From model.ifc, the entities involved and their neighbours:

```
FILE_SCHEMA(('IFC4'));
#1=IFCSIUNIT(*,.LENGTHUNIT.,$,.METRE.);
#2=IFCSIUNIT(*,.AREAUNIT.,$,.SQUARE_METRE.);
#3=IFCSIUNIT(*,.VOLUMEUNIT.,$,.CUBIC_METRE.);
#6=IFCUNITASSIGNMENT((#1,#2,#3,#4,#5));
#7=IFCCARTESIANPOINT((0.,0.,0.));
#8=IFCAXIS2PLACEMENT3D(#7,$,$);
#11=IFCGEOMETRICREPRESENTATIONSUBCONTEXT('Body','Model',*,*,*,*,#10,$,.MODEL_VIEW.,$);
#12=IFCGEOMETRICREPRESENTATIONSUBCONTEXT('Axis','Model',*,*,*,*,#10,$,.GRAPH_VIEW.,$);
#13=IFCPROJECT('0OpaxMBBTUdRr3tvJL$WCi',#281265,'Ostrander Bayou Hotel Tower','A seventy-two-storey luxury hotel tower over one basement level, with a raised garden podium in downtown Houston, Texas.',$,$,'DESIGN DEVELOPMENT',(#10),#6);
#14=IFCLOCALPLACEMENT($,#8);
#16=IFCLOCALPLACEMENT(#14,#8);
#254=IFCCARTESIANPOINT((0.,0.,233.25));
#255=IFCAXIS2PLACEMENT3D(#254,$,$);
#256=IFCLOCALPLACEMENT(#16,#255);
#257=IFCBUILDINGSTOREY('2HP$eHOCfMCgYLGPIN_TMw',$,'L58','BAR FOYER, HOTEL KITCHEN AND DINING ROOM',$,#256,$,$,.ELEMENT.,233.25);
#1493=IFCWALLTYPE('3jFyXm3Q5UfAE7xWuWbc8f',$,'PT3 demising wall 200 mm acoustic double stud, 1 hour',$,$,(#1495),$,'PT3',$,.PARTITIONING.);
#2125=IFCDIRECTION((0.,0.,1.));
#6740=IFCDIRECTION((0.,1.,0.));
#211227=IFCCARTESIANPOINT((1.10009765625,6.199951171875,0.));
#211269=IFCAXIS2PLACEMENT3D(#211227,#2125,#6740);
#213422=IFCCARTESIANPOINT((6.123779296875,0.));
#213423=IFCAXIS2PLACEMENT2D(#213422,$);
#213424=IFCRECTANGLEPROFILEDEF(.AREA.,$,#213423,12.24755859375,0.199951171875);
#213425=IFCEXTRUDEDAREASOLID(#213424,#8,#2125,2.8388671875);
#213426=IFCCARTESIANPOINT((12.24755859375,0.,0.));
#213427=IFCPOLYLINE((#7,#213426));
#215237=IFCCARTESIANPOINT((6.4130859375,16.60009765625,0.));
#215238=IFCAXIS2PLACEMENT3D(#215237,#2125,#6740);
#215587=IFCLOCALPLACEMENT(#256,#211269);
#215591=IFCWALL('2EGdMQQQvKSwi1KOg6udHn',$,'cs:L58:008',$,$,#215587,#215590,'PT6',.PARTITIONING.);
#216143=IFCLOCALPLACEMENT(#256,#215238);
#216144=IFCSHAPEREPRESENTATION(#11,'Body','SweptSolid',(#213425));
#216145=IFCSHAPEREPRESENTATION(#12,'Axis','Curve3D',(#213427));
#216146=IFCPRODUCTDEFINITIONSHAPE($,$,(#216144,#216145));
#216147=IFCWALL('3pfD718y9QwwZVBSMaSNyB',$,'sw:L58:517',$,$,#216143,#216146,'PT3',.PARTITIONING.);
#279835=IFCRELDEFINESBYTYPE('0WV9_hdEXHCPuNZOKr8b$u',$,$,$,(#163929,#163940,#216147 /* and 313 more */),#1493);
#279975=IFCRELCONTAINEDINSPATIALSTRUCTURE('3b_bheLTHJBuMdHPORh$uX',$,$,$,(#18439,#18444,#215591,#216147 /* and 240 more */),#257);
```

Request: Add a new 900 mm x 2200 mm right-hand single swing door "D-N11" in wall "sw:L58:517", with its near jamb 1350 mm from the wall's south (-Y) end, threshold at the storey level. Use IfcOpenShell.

```python
import numpy as np
import ifcopenshell
import ifcopenshell.api.feature
import ifcopenshell.api.geometry
import ifcopenshell.api.root
import ifcopenshell.api.spatial
import ifcopenshell.geom
import ifcopenshell.util.element
import ifcopenshell.util.placement
import ifcopenshell.util.representation
import ifcopenshell.util.shape
import ifcopenshell.util.unit

model = ifcopenshell.open("model.ifc")
unit_scale = ifcopenshell.util.unit.calculate_unit_scale(model)
settings = ifcopenshell.geom.settings()


def volume(element):
    """Net volume in cubic metres, openings subtracted."""
    shape = ifcopenshell.geom.create_shape(settings, element)
    return ifcopenshell.util.shape.get_volume(shape.geometry)


wall = model.by_guid("3pfD718y9QwwZVBSMaSNyB")
storey = ifcopenshell.util.element.get_container(wall, ifc_class="IfcBuildingStorey")
context = ifcopenshell.util.representation.get_context(model, "Model", "Body", "MODEL_VIEW")
before = volume(wall)

width, height, from_end, sill = 0.9, 2.2, 1.35, 0.0  # metres

# The wall runs along its own X axis, and the end named is its -X end.
wall_shape = ifcopenshell.geom.create_shape(settings, wall)
x, y, z = ifcopenshell.util.shape.get_vertices(wall_shape.geometry).T
start = x.min() + from_end
face, thickness = float(y.min()), float(y.max() - y.min())
wall_matrix = ifcopenshell.util.placement.get_local_placement(wall.ObjectPlacement)
level = ifcopenshell.util.placement.get_local_placement(storey.ObjectPlacement)[2, 3]


def in_wall(x, y):
    """Placement at x, y metres in the wall's axes, at sill height."""
    matrix = wall_matrix.copy()
    matrix[:, 3] = wall_matrix @ np.array([x / unit_scale, y / unit_scale, 0.0, 1.0])
    matrix[2, 3] = level + sill / unit_scale
    return matrix


# Opening: a box that overshoots both wall faces by 50 mm.
opening = ifcopenshell.api.root.create_entity(model, ifc_class="IfcOpeningElement", predefined_type="OPENING")
box = ifcopenshell.api.geometry.add_wall_representation(
    model, context=context, length=width, height=height, thickness=thickness + 0.1
)
ifcopenshell.api.geometry.assign_representation(model, product=opening, representation=box)
ifcopenshell.api.geometry.edit_object_placement(model, product=opening, matrix=in_wall(start, face - 0.05), is_si=False)
ifcopenshell.api.feature.add_feature(model, feature=opening, element=wall)

door = ifcopenshell.api.root.create_entity(model, ifc_class="IfcDoor", name="D-N11", predefined_type="DOOR")
door.OverallWidth, door.OverallHeight = width / unit_scale, height / unit_scale
door.OperationType = "SINGLE_SWING_RIGHT"
body = ifcopenshell.api.geometry.add_door_representation(
    model,
    context=context,
    overall_width=door.OverallWidth,
    overall_height=door.OverallHeight,
    operation_type="SINGLE_SWING_RIGHT",
    lining_properties={"LiningDepth": thickness / unit_scale, "ThresholdDepth": thickness / unit_scale},
)
ifcopenshell.api.geometry.assign_representation(model, product=door, representation=body)
ifcopenshell.api.spatial.assign_container(model, products=[door], relating_structure=storey)
ifcopenshell.api.feature.add_filling(model, opening=opening, element=door)

# The lining spans the wall, so the door starts at the wall face.
ifcopenshell.api.geometry.edit_object_placement(model, product=door, matrix=in_wall(start, face), is_si=False)

after = volume(wall)

print(f"wall volume {before:.3f} -> {after:.3f} m3")

model.write("model_rev.ifc")
```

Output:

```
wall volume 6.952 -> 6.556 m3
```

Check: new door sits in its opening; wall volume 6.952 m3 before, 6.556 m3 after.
